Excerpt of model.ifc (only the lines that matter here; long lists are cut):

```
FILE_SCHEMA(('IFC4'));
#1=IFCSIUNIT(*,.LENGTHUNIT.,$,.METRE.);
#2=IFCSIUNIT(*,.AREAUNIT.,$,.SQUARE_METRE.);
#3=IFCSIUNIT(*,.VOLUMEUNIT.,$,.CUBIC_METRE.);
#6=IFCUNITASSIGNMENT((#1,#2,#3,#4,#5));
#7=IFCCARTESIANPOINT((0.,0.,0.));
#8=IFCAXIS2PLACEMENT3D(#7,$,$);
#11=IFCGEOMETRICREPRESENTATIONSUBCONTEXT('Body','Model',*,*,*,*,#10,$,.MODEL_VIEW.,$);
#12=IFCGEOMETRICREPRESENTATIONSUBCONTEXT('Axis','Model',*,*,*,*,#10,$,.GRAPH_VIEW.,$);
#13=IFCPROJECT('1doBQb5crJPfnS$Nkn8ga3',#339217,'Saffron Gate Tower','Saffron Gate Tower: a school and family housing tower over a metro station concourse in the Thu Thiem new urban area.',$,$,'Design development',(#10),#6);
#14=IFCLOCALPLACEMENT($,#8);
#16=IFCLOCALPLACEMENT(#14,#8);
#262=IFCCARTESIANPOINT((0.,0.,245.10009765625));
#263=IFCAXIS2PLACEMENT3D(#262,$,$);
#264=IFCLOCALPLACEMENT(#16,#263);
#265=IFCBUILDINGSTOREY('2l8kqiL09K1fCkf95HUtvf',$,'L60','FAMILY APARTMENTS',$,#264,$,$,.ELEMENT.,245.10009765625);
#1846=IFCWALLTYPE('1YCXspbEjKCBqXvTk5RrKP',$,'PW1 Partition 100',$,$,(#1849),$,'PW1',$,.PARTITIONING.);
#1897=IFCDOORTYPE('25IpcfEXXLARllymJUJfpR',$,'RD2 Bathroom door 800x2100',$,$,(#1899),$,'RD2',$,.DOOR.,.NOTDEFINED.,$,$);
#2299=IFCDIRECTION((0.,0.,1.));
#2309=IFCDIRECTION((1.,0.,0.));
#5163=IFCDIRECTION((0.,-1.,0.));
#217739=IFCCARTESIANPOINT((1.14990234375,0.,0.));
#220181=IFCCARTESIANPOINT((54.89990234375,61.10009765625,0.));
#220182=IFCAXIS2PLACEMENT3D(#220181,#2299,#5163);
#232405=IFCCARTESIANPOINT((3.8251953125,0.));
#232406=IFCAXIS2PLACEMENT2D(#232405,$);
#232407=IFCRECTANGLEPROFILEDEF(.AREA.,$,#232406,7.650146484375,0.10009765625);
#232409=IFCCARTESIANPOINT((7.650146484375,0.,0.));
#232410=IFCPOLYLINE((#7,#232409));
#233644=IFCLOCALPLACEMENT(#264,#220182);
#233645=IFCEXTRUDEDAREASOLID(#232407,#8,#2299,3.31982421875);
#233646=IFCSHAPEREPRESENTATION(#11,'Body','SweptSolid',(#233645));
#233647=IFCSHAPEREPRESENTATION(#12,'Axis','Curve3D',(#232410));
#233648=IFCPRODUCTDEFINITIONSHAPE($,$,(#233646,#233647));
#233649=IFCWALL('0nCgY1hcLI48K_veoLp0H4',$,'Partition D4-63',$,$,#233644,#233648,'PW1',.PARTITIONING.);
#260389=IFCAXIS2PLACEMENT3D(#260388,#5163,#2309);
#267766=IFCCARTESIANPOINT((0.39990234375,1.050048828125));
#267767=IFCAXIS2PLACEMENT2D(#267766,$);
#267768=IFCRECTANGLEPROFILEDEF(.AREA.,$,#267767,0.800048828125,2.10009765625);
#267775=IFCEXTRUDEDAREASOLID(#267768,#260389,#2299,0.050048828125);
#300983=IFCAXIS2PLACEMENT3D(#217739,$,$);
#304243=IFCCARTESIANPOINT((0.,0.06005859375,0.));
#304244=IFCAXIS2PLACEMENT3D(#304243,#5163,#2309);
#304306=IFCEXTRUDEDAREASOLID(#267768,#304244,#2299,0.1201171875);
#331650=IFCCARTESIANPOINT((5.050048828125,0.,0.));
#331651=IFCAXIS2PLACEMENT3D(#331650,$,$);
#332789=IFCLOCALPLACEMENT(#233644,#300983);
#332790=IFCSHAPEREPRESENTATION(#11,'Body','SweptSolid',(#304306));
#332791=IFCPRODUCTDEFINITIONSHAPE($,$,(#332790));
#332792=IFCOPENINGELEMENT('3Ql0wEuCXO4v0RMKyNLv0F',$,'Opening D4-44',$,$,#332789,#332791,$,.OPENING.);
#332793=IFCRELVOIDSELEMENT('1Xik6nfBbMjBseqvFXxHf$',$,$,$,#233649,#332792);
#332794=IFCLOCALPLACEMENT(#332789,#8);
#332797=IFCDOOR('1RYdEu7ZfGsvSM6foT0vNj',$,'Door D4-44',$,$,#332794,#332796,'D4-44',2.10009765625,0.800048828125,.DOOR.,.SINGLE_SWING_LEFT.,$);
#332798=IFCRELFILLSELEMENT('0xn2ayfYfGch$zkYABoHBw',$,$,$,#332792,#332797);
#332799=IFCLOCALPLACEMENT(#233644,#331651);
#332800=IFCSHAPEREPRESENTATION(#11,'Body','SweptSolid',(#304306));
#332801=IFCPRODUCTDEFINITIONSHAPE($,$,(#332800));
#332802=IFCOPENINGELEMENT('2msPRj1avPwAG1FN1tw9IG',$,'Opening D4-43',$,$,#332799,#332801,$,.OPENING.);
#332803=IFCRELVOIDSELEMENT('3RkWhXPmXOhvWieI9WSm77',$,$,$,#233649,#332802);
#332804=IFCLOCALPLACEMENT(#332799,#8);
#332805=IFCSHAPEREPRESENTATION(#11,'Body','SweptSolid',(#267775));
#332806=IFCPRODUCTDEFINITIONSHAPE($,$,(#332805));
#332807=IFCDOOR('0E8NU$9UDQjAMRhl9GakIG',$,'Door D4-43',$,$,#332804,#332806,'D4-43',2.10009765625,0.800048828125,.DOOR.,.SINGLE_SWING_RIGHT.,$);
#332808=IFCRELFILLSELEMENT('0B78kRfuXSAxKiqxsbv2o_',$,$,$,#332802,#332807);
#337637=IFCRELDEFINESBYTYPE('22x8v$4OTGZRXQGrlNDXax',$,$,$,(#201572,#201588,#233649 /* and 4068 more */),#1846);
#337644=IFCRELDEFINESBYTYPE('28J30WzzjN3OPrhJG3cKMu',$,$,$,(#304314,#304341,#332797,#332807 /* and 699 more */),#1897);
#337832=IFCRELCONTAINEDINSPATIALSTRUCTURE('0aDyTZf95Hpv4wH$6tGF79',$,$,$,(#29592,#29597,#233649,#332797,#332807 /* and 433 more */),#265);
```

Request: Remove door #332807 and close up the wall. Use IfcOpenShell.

```python
import ifcopenshell
import ifcopenshell.api.feature
import ifcopenshell.api.root
import ifcopenshell.geom
import ifcopenshell.util.shape

model = ifcopenshell.open("model.ifc")
settings = ifcopenshell.geom.settings()


def volume(element):
    """Net volume in cubic metres, openings subtracted."""
    shape = ifcopenshell.geom.create_shape(settings, element)
    return ifcopenshell.util.shape.get_volume(shape.geometry)


door = model.by_id(332807)
opening = door.FillsVoids[0].RelatingOpeningElement
wall = opening.VoidsElements[0].RelatingBuildingElement
before = volume(wall)

ifcopenshell.api.root.remove_product(model, product=door)
ifcopenshell.api.feature.remove_feature(model, feature=opening)

after = volume(wall)

print(f"wall volume {before:.3f} -> {after:.3f} m3")

model.write("model_rev.ifc")
```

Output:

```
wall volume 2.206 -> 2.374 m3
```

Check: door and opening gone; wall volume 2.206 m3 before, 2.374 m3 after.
